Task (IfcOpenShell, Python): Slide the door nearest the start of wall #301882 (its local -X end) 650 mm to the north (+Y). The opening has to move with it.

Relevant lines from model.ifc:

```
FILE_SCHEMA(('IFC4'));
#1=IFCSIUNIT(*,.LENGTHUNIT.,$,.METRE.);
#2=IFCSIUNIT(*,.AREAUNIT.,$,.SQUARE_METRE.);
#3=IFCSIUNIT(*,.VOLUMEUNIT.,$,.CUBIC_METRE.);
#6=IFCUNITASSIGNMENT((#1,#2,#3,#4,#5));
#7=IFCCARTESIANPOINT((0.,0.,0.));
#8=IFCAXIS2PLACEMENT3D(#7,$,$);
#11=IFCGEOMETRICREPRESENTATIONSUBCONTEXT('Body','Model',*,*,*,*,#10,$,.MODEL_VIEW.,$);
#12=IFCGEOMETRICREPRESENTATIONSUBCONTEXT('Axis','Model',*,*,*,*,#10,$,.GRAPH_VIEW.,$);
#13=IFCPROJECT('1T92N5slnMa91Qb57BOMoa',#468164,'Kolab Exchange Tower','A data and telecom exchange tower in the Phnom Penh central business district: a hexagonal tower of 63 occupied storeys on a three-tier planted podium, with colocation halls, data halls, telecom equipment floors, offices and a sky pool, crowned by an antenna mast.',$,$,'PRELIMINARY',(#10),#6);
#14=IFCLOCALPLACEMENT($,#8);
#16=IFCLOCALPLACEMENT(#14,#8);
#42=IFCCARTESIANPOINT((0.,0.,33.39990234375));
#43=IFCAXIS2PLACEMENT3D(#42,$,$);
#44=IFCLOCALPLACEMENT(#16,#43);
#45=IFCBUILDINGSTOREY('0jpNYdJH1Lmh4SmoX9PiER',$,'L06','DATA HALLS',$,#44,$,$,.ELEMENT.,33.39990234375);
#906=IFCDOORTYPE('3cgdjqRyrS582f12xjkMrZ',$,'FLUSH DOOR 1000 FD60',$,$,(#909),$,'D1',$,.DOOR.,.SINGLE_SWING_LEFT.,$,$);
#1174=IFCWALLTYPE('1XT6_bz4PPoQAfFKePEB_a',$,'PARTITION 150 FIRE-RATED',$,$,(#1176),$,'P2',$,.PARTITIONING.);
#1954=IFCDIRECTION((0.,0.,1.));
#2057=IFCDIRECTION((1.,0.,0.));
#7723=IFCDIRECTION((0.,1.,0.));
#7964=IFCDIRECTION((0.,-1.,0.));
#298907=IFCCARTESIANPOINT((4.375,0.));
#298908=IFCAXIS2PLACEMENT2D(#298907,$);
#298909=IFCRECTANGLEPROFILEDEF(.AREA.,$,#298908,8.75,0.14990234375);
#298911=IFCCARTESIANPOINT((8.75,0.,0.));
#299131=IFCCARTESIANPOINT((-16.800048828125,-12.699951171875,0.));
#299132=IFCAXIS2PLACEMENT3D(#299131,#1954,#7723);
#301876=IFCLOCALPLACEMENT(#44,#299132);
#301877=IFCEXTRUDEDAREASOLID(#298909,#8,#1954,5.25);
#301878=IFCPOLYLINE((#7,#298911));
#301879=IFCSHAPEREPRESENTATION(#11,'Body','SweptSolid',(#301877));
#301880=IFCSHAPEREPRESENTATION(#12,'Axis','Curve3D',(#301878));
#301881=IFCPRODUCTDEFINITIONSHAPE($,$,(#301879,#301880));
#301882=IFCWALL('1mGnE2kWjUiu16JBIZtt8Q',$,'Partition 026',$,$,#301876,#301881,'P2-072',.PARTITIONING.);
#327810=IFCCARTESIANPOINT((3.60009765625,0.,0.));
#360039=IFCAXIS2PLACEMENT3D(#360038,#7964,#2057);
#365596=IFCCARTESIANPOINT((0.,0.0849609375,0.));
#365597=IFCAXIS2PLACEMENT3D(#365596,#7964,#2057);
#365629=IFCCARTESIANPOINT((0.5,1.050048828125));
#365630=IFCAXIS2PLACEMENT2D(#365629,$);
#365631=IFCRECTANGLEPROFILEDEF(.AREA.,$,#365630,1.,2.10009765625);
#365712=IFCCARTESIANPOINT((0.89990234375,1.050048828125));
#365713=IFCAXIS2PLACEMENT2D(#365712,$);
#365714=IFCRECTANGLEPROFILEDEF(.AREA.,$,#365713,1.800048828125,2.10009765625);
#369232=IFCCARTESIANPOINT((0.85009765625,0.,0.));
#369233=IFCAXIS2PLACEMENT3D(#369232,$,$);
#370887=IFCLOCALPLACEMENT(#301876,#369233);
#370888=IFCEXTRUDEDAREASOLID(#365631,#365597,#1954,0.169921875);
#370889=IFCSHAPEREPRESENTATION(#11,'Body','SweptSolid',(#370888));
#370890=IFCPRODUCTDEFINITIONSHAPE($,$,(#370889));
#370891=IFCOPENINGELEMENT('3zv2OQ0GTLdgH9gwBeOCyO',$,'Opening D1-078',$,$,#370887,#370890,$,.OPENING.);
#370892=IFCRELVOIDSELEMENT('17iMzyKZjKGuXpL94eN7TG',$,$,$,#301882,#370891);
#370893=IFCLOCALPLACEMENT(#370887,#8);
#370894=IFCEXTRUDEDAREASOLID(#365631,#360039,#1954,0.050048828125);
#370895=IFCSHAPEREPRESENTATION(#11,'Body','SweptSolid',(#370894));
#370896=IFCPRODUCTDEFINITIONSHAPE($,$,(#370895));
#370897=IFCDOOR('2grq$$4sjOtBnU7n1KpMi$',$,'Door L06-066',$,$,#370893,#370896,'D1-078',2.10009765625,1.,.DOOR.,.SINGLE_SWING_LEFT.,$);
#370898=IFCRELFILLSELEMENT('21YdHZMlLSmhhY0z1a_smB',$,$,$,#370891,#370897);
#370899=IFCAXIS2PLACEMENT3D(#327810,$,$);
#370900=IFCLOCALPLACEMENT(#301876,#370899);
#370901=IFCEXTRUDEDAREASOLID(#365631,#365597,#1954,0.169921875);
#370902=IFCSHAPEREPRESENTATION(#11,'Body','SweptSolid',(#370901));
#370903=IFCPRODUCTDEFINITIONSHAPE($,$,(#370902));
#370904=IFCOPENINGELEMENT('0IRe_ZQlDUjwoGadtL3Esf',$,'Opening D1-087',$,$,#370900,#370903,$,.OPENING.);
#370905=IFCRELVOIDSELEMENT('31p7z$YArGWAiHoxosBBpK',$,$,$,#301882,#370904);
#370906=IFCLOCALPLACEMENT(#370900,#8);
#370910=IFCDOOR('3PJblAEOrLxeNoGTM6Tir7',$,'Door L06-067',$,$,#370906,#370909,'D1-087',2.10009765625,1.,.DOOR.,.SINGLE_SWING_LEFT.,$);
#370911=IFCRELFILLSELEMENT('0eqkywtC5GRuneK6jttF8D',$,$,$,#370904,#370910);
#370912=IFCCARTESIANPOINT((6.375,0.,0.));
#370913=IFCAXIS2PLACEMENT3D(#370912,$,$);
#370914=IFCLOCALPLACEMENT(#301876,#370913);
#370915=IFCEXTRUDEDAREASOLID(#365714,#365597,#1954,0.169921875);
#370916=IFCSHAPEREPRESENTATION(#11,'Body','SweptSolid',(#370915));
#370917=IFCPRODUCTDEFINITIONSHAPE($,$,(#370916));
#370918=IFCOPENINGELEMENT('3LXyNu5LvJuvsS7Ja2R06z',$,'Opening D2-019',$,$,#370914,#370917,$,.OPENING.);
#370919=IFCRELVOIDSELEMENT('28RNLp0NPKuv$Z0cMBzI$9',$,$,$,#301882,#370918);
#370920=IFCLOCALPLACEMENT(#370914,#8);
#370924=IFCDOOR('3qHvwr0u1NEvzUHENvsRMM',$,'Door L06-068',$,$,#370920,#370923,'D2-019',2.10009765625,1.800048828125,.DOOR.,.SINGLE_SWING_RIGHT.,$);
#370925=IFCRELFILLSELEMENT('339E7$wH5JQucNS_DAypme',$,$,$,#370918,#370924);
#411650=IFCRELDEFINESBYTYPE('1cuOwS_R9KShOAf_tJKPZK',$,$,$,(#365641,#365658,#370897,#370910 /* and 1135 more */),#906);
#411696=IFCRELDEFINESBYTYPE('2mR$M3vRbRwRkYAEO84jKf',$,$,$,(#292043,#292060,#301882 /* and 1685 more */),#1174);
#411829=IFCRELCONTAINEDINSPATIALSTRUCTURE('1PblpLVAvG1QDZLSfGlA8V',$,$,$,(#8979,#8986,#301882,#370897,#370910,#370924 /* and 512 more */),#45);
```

```python
import ifcopenshell
import ifcopenshell.api.geometry
import ifcopenshell.util.placement
import ifcopenshell.util.unit

model = ifcopenshell.open("model.ifc")
unit_scale = ifcopenshell.util.unit.calculate_unit_scale(model)

door = model.by_guid("2grq$$4sjOtBnU7n1KpMi$")
opening = door.FillsVoids[0].RelatingOpeningElement
wall = opening.VoidsElements[0].RelatingBuildingElement

wall_matrix = ifcopenshell.util.placement.get_local_placement(wall.ObjectPlacement)
shift = wall_matrix[:3, 0] * 0.65 / unit_scale
before = ifcopenshell.util.placement.get_local_placement(door.ObjectPlacement)[:3, 3].copy()

# The door is placed relative to its opening, so it follows when the opening moves.
matrix = ifcopenshell.util.placement.get_local_placement(opening.ObjectPlacement)
matrix[:3, 3] += shift
ifcopenshell.api.geometry.edit_object_placement(
    model, product=opening, matrix=matrix, is_si=False, should_transform_children=True
)

after = ifcopenshell.util.placement.get_local_placement(door.ObjectPlacement)[:3, 3]
print("door moved by", (after - before).round(3) + 0.0)

model.write("model_updated.ifc")
```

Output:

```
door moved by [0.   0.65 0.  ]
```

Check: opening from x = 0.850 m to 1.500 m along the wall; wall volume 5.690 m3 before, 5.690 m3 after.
